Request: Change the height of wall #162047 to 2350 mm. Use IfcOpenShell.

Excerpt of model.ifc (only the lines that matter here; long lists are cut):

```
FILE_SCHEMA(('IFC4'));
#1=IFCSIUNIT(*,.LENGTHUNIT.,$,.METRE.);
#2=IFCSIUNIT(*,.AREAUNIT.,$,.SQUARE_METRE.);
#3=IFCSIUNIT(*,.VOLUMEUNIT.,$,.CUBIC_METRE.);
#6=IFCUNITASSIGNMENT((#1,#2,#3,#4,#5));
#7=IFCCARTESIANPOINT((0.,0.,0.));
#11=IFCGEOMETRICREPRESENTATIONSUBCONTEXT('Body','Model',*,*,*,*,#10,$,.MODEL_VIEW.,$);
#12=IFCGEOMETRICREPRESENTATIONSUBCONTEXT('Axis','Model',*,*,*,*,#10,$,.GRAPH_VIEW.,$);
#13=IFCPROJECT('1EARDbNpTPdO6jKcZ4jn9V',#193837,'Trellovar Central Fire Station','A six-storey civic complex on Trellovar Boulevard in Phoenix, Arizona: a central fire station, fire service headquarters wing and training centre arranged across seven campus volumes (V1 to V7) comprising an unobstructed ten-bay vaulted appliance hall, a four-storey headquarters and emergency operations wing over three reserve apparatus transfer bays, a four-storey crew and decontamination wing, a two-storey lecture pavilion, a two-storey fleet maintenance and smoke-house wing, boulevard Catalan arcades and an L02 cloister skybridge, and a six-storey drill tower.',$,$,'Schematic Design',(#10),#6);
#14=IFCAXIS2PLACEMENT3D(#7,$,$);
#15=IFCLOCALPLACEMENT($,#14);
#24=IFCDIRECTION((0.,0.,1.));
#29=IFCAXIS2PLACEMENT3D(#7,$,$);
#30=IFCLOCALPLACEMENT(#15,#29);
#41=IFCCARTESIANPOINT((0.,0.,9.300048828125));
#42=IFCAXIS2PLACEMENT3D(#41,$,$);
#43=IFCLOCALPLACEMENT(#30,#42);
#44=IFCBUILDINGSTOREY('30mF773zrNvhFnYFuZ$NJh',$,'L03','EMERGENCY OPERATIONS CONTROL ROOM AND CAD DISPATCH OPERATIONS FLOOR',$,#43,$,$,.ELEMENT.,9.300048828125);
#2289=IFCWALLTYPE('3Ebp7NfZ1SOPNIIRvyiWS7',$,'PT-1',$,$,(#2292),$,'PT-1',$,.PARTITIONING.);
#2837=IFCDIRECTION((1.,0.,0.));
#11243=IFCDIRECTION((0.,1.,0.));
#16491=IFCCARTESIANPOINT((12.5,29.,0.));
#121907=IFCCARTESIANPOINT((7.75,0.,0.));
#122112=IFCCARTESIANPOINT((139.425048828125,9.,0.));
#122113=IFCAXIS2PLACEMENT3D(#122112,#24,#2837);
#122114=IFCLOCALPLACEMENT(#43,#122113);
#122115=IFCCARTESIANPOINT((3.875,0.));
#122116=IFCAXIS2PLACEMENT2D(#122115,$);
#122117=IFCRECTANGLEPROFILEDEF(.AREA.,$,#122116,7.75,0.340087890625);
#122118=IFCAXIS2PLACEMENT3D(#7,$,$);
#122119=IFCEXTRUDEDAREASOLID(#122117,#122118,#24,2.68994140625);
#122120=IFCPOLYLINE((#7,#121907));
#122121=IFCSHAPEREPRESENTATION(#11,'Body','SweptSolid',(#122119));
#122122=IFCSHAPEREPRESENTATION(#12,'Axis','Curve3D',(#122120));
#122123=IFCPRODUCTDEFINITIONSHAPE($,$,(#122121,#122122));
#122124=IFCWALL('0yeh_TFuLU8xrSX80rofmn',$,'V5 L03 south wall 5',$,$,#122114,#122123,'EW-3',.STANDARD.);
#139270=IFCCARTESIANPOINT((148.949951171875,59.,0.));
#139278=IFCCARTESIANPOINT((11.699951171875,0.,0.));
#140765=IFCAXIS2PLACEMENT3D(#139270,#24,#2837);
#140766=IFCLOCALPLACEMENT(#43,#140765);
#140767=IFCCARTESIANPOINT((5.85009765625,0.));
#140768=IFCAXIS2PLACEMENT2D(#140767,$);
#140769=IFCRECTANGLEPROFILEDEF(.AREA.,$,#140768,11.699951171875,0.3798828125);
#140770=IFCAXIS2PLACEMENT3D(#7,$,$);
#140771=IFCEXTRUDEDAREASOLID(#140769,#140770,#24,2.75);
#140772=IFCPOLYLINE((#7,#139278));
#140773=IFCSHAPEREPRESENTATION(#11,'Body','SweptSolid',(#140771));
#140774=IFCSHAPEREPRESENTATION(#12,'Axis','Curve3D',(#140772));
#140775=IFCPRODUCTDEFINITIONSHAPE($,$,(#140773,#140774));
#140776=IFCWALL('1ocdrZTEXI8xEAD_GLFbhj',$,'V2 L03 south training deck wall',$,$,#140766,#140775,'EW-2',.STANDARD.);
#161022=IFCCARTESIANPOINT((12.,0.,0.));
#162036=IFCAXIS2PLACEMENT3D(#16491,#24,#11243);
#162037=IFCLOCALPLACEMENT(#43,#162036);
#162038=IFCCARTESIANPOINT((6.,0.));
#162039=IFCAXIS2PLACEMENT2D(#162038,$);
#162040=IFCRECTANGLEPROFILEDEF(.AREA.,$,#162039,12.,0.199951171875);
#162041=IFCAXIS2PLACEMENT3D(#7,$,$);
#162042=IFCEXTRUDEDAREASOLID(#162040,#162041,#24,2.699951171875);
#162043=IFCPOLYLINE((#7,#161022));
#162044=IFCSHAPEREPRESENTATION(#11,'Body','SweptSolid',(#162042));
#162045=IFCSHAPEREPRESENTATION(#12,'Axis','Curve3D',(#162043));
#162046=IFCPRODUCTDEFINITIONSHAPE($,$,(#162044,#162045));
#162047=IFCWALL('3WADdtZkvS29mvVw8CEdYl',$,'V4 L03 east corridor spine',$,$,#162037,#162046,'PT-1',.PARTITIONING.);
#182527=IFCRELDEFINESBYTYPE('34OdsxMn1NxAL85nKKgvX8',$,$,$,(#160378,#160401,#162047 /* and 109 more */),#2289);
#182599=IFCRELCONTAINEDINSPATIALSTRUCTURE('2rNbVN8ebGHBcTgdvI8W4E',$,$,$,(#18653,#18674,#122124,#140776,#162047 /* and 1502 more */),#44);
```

```python
import ifcopenshell
import ifcopenshell.geom
import ifcopenshell.util.representation
import ifcopenshell.util.shape

model = ifcopenshell.open("model.ifc")
settings = ifcopenshell.geom.settings()


def volume(element):
    """Net volume in cubic metres, openings subtracted."""
    shape = ifcopenshell.geom.create_shape(settings, element)
    return ifcopenshell.util.shape.get_volume(shape.geometry)


wall = model.by_id(162047)
before = volume(wall)

body = ifcopenshell.util.representation.get_representation(wall, "Model", "Body")
solid = body.Items[0]
old_height = solid.Depth
solid.Depth = 2.35
after = volume(wall)

print(f"height {old_height:g} -> {solid.Depth:g}, volume {before:.3f} -> {after:.3f} m3")

model.write("model-out.ifc")
```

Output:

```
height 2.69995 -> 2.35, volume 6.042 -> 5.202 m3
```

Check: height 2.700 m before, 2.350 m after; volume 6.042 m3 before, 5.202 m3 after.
